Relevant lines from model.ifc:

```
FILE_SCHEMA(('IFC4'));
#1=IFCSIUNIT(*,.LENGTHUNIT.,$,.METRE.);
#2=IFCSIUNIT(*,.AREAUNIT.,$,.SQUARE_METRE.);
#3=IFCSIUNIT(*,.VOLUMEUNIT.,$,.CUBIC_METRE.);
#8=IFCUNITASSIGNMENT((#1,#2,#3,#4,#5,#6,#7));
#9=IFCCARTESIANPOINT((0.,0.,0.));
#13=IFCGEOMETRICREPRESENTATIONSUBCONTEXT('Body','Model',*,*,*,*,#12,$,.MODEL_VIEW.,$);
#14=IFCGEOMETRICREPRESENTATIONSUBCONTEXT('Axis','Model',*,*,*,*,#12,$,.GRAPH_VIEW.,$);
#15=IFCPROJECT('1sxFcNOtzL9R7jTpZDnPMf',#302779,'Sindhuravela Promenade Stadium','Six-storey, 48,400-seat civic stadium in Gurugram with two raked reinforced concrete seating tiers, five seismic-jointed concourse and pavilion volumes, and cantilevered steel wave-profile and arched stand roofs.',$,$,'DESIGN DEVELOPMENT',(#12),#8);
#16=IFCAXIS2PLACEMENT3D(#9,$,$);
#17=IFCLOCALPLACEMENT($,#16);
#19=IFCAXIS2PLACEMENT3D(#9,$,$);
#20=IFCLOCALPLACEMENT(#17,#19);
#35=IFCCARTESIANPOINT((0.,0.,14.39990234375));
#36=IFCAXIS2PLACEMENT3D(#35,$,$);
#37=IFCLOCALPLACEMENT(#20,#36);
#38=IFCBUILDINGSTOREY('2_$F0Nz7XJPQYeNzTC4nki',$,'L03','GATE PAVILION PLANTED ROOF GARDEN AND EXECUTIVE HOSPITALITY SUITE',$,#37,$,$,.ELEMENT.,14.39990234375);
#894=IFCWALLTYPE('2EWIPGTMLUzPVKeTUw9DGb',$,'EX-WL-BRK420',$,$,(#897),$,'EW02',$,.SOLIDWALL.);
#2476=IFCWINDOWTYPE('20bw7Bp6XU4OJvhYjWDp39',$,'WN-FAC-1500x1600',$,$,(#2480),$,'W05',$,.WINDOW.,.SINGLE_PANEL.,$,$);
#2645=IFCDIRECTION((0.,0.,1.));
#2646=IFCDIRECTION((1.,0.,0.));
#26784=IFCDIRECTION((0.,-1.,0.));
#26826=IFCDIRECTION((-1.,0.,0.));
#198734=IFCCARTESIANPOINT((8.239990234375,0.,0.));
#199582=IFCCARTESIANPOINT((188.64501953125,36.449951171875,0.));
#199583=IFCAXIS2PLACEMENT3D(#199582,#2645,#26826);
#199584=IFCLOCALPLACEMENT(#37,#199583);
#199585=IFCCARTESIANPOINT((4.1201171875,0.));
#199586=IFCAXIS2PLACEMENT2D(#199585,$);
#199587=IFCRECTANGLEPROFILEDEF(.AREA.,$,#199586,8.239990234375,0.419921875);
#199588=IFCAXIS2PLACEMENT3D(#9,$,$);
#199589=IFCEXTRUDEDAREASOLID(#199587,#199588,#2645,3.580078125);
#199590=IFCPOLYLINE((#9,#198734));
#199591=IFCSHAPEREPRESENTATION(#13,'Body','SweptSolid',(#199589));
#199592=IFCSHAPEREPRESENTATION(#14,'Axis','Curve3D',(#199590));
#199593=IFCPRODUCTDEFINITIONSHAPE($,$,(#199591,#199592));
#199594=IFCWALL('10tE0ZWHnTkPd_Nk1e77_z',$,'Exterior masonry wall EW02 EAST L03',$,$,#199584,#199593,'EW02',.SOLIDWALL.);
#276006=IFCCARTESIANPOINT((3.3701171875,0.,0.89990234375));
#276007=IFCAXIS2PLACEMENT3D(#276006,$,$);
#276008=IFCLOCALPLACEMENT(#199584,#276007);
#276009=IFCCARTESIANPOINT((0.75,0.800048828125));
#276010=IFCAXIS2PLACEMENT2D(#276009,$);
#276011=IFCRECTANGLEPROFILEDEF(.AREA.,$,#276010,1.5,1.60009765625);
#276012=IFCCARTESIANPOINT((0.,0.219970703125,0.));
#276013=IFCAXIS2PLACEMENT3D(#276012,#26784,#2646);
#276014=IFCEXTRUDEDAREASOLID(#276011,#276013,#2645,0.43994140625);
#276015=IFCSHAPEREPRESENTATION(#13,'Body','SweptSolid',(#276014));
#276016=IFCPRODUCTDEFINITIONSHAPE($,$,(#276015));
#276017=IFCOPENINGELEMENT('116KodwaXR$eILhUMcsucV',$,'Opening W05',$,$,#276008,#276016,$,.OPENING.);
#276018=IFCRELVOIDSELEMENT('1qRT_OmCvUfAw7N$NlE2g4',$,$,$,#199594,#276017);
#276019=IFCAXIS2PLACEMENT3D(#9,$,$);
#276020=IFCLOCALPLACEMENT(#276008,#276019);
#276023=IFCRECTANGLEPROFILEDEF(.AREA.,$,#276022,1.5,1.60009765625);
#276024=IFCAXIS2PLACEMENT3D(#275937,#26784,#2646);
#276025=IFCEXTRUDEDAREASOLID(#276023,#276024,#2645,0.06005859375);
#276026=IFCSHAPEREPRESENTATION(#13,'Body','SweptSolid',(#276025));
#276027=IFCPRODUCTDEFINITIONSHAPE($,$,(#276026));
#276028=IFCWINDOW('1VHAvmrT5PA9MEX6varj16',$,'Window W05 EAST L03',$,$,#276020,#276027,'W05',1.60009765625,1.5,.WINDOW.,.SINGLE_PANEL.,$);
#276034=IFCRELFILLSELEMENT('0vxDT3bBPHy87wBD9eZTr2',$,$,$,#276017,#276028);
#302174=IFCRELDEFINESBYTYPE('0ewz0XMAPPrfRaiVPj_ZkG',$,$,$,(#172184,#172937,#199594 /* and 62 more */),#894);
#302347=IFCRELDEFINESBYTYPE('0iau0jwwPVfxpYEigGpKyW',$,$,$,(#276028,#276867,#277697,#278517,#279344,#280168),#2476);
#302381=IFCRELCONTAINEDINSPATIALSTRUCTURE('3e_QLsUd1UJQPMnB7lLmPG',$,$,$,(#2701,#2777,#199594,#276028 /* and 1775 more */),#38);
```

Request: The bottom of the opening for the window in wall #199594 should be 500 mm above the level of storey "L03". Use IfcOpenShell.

```python
import numpy as np
import ifcopenshell
import ifcopenshell.api.geometry
import ifcopenshell.geom
import ifcopenshell.util.element
import ifcopenshell.util.placement
import ifcopenshell.util.shape
import ifcopenshell.util.unit

model = ifcopenshell.open("model.ifc")
unit_scale = ifcopenshell.util.unit.calculate_unit_scale(model)

window = model.by_guid("1VHAvmrT5PA9MEX6varj16")
opening = window.FillsVoids[0].RelatingOpeningElement
storey = ifcopenshell.util.element.get_container(window, ifc_class="IfcBuildingStorey")
level = ifcopenshell.util.placement.get_local_placement(storey.ObjectPlacement)[2, 3]

# The opening's origin need not be at the sill, so measure its lowest point.
shape = ifcopenshell.geom.create_shape(ifcopenshell.geom.settings(), opening)
bottom = ifcopenshell.util.shape.get_shape_bottom_elevation(shape, shape.geometry) / unit_scale
dz = level + 0.5 / unit_scale - bottom

shift = np.array([0.0, 0.0, dz])
# The window is placed relative to its opening, so it follows when the opening moves.
matrix = ifcopenshell.util.placement.get_local_placement(opening.ObjectPlacement)
matrix[:3, 3] += shift
ifcopenshell.api.geometry.edit_object_placement(
    model, product=opening, matrix=matrix, is_si=False, should_transform_children=True
)

print(f"moved by {dz * unit_scale:+.3f} m")

model.write("model_edited.ifc")
```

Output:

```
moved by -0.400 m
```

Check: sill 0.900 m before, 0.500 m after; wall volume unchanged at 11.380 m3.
